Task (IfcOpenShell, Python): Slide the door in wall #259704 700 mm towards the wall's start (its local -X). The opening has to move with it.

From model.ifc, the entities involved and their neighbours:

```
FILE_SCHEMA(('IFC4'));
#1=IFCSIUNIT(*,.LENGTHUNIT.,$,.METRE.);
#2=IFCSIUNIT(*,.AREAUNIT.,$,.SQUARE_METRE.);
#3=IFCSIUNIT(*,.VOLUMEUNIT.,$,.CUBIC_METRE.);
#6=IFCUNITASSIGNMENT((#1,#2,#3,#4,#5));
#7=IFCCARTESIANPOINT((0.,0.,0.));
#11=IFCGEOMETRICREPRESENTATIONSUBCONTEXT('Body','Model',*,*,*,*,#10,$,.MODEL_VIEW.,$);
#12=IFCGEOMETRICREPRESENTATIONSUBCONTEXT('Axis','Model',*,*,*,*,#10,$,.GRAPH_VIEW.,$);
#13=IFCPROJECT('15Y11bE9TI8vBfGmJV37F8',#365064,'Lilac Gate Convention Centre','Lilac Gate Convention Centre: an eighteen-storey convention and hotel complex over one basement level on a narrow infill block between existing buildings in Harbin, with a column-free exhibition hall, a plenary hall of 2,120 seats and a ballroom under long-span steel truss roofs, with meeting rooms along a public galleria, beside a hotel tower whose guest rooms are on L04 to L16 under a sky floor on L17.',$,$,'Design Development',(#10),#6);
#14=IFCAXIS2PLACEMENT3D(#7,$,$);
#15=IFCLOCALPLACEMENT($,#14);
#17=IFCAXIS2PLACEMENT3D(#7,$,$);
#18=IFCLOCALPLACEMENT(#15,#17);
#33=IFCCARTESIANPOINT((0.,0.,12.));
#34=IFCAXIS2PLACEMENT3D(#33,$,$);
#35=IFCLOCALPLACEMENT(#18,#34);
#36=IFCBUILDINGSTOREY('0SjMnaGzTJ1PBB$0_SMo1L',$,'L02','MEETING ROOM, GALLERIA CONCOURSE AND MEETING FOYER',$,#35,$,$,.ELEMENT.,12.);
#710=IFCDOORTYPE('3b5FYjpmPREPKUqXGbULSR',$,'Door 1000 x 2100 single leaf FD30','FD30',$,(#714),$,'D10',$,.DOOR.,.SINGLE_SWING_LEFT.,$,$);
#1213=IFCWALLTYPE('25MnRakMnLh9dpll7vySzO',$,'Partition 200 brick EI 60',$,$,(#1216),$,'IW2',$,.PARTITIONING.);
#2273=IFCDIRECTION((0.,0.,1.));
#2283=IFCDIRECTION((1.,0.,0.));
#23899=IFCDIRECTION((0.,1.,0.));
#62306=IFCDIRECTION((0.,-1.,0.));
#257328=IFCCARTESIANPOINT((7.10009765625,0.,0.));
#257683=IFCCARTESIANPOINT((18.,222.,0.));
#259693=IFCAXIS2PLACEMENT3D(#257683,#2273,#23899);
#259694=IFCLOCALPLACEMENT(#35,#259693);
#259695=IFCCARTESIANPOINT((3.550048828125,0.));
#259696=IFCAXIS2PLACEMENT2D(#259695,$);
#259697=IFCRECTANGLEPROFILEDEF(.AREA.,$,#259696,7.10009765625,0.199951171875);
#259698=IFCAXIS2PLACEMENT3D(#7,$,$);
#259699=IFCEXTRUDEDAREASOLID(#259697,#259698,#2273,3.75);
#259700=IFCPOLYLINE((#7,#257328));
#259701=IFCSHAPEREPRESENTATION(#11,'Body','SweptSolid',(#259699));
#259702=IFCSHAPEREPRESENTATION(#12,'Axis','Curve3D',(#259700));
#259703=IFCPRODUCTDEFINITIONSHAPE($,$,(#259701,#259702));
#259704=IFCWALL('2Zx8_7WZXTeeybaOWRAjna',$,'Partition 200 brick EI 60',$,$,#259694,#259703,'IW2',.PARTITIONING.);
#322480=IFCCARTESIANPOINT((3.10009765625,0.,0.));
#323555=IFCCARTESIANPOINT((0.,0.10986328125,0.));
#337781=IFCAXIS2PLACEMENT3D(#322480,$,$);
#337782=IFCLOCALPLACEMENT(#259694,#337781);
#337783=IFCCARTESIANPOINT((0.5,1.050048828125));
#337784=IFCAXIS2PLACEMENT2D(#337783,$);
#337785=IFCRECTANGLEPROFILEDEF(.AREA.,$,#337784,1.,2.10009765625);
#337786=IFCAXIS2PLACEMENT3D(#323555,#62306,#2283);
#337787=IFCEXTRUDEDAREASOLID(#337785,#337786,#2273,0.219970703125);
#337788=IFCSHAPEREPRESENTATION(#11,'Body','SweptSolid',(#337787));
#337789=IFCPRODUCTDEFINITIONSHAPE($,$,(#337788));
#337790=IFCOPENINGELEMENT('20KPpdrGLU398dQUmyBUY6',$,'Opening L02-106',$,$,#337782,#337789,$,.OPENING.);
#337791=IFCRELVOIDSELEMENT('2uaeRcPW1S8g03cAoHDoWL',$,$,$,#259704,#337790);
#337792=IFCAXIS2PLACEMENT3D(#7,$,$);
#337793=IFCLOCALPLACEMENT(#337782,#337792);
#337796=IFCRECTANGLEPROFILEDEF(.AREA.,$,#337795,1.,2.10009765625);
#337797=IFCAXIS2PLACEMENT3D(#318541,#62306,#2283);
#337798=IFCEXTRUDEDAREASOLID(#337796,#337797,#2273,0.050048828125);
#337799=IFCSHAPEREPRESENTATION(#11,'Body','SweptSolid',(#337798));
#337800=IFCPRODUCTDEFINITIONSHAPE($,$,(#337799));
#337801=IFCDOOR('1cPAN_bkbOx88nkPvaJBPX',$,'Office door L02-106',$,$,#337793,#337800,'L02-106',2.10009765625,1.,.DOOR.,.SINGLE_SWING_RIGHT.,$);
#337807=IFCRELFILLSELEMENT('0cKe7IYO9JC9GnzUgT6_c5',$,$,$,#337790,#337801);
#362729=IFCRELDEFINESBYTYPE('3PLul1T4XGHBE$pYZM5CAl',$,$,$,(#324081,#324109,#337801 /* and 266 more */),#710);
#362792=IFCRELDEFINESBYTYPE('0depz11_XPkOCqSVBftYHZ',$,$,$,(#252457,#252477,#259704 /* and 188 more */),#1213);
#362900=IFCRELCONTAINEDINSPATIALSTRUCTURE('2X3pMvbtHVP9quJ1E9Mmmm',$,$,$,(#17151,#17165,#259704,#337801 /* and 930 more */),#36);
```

```python
import ifcopenshell
import ifcopenshell.api.geometry
import ifcopenshell.util.placement
import ifcopenshell.util.unit

model = ifcopenshell.open("model.ifc")
unit_scale = ifcopenshell.util.unit.calculate_unit_scale(model)

door = model.by_id(337801)
opening = door.FillsVoids[0].RelatingOpeningElement
wall = opening.VoidsElements[0].RelatingBuildingElement

wall_matrix = ifcopenshell.util.placement.get_local_placement(wall.ObjectPlacement)
shift = wall_matrix[:3, 0] * -0.7 / unit_scale
before = ifcopenshell.util.placement.get_local_placement(door.ObjectPlacement)[:3, 3].copy()

# The door is placed relative to its opening, so it follows when the opening moves.
matrix = ifcopenshell.util.placement.get_local_placement(opening.ObjectPlacement)
matrix[:3, 3] += shift
ifcopenshell.api.geometry.edit_object_placement(
    model, product=opening, matrix=matrix, is_si=False, should_transform_children=True
)

after = ifcopenshell.util.placement.get_local_placement(door.ObjectPlacement)[:3, 3]
print("door moved by", (after - before).round(3) + 0.0)

model.write("model_v2.ifc")
```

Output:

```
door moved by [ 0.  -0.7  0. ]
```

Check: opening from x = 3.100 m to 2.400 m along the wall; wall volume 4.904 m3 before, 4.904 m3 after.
